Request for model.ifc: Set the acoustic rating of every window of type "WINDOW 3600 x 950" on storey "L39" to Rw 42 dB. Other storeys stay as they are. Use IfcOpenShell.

First a look at what the model holds.

```python
import ifcopenshell
import ifcopenshell.util.element

model = ifcopenshell.open("model.ifc")
print(model.schema)
storey = next(s for s in model.by_type("IfcBuildingStorey") if s.Name == "L39")
windows = [e for e in ifcopenshell.util.element.get_decomposition(storey) if e.is_a("IfcWindow")]
seen = {}
for e in windows:
    element_type = ifcopenshell.util.element.get_type(e)
    key = (element_type.Name if element_type != e and element_type else None, ifcopenshell.util.element.get_pset(e, "Pset_WindowCommon", "AcousticRating"))
    seen[key] = seen.get(key, 0) + 1
for (name, value), count in sorted(seen.items(), key=str):
    print(count, "x", name, "|", value)
```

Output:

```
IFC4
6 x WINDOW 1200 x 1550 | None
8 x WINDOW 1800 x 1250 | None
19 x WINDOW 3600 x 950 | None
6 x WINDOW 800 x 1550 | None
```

```python
import ifcopenshell
import ifcopenshell.api.pset
import ifcopenshell.util.element

model = ifcopenshell.open("model.ifc")

storey = next(s for s in model.by_type("IfcBuildingStorey") if s.Name == "L39")
windows = [e for e in ifcopenshell.util.element.get_decomposition(storey) if e.is_a("IfcWindow")]

count = 0
for e in windows:
    element_type = ifcopenshell.util.element.get_type(e)
    if element_type in (None, e) or element_type.Name != "WINDOW 3600 x 950":
        continue
    found = ifcopenshell.util.element.get_pset(e, "Pset_WindowCommon", should_inherit=False)
    if found:
        pset = model.by_id(found["id"])
        if len(ifcopenshell.util.element.get_elements_by_pset(pset)) > 1:
            pset = ifcopenshell.api.pset.unshare_pset(model, products=[e], pset=pset)[0]
    else:
        pset = ifcopenshell.api.pset.add_pset(model, product=e, name="Pset_WindowCommon")
    ifcopenshell.api.pset.edit_pset(model, pset=pset, properties={"AcousticRating": "Rw 42 dB"})
    count += 1

print(count, "windows updated")

model.write("model-out.ifc")
```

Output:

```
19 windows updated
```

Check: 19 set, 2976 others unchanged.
